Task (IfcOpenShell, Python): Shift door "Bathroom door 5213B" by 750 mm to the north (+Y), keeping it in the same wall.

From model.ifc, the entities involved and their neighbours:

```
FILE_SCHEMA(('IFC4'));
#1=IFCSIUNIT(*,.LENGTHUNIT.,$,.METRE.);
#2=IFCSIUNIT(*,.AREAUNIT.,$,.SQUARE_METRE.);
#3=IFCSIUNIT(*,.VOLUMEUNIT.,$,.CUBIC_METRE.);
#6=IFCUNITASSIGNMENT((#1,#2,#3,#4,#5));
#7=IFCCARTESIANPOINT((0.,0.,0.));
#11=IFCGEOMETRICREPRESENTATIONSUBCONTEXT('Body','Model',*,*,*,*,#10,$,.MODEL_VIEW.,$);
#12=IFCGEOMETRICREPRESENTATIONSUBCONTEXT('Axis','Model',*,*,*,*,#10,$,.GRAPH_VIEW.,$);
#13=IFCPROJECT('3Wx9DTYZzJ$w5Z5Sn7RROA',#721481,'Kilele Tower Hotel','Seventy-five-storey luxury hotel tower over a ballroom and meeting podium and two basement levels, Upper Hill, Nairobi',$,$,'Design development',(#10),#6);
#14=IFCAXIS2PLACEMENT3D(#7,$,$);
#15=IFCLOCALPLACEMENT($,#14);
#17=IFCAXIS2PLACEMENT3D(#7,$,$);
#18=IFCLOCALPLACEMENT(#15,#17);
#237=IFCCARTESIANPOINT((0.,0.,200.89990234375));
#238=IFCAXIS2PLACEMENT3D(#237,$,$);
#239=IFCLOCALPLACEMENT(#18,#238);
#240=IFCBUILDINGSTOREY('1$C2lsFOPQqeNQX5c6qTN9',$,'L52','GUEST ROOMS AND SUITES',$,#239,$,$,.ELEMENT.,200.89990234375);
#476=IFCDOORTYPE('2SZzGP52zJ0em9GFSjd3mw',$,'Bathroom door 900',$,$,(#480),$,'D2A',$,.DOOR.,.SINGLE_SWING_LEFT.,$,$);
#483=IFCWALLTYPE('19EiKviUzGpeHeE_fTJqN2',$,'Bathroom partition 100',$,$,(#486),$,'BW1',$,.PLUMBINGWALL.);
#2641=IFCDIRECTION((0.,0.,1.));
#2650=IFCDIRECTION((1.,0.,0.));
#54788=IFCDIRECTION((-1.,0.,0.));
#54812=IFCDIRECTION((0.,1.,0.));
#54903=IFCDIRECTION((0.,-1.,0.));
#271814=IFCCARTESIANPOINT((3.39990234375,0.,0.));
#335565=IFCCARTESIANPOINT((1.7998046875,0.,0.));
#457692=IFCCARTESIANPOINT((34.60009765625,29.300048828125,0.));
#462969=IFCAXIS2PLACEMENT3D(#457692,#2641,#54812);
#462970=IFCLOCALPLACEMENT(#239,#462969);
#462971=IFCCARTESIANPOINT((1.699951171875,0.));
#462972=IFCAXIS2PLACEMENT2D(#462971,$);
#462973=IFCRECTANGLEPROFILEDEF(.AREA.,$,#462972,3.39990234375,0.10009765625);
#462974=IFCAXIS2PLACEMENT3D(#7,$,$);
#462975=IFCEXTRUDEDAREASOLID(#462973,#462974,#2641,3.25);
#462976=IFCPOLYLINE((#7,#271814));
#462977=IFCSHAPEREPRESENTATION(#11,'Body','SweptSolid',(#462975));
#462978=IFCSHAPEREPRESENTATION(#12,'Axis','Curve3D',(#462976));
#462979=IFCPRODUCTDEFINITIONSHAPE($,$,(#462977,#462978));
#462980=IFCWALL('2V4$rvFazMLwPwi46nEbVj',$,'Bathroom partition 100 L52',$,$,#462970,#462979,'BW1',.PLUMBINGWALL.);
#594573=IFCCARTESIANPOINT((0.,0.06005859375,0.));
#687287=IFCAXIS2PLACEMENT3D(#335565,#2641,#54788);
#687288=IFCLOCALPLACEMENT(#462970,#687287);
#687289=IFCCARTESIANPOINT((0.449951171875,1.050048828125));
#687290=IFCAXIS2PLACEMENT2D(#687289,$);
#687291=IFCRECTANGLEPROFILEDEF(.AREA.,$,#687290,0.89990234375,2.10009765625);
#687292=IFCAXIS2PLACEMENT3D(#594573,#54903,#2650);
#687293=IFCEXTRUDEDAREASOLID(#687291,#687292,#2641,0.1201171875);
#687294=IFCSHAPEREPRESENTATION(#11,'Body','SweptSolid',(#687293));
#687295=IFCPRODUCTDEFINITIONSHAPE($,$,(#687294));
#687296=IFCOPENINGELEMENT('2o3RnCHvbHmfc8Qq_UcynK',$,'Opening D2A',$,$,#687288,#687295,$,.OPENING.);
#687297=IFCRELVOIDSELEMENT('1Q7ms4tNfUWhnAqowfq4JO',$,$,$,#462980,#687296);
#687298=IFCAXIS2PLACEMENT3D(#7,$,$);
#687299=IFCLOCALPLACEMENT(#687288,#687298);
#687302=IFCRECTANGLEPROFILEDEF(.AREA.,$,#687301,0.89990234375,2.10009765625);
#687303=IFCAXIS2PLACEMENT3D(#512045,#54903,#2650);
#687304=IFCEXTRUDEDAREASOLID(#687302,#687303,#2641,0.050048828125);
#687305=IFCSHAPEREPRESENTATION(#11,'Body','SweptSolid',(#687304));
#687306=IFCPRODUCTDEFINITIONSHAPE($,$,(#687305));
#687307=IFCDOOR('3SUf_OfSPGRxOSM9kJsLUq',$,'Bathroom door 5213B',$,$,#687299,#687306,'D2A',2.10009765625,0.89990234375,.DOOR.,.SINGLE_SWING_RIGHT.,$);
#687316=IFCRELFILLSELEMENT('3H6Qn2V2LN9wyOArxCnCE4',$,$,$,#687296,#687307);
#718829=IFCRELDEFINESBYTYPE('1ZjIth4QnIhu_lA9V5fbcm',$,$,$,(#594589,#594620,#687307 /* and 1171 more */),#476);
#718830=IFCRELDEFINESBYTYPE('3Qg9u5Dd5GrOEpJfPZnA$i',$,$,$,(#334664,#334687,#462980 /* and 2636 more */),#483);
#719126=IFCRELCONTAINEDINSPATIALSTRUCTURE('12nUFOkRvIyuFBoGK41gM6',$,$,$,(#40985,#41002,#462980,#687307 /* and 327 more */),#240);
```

```python
import ifcopenshell
import ifcopenshell.api.geometry
import ifcopenshell.util.placement

model = ifcopenshell.open("model.ifc")

door = model.by_guid("3SUf_OfSPGRxOSM9kJsLUq")
opening = door.FillsVoids[0].RelatingOpeningElement
wall = opening.VoidsElements[0].RelatingBuildingElement

wall_matrix = ifcopenshell.util.placement.get_local_placement(wall.ObjectPlacement)
shift = wall_matrix[:3, 0] * 0.75
before = ifcopenshell.util.placement.get_local_placement(door.ObjectPlacement)[:3, 3].copy()

# The door is placed relative to its opening, so it follows when the opening moves.
matrix = ifcopenshell.util.placement.get_local_placement(opening.ObjectPlacement)
matrix[:3, 3] += shift
ifcopenshell.api.geometry.edit_object_placement(
    model, product=opening, matrix=matrix, is_si=False, should_transform_children=True
)

after = ifcopenshell.util.placement.get_local_placement(door.ObjectPlacement)[:3, 3]
print("door moved by", (after - before).round(3) + 0.0)

model.write("model-out.ifc")
```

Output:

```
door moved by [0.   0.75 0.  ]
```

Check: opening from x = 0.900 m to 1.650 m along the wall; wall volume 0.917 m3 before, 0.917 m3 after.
